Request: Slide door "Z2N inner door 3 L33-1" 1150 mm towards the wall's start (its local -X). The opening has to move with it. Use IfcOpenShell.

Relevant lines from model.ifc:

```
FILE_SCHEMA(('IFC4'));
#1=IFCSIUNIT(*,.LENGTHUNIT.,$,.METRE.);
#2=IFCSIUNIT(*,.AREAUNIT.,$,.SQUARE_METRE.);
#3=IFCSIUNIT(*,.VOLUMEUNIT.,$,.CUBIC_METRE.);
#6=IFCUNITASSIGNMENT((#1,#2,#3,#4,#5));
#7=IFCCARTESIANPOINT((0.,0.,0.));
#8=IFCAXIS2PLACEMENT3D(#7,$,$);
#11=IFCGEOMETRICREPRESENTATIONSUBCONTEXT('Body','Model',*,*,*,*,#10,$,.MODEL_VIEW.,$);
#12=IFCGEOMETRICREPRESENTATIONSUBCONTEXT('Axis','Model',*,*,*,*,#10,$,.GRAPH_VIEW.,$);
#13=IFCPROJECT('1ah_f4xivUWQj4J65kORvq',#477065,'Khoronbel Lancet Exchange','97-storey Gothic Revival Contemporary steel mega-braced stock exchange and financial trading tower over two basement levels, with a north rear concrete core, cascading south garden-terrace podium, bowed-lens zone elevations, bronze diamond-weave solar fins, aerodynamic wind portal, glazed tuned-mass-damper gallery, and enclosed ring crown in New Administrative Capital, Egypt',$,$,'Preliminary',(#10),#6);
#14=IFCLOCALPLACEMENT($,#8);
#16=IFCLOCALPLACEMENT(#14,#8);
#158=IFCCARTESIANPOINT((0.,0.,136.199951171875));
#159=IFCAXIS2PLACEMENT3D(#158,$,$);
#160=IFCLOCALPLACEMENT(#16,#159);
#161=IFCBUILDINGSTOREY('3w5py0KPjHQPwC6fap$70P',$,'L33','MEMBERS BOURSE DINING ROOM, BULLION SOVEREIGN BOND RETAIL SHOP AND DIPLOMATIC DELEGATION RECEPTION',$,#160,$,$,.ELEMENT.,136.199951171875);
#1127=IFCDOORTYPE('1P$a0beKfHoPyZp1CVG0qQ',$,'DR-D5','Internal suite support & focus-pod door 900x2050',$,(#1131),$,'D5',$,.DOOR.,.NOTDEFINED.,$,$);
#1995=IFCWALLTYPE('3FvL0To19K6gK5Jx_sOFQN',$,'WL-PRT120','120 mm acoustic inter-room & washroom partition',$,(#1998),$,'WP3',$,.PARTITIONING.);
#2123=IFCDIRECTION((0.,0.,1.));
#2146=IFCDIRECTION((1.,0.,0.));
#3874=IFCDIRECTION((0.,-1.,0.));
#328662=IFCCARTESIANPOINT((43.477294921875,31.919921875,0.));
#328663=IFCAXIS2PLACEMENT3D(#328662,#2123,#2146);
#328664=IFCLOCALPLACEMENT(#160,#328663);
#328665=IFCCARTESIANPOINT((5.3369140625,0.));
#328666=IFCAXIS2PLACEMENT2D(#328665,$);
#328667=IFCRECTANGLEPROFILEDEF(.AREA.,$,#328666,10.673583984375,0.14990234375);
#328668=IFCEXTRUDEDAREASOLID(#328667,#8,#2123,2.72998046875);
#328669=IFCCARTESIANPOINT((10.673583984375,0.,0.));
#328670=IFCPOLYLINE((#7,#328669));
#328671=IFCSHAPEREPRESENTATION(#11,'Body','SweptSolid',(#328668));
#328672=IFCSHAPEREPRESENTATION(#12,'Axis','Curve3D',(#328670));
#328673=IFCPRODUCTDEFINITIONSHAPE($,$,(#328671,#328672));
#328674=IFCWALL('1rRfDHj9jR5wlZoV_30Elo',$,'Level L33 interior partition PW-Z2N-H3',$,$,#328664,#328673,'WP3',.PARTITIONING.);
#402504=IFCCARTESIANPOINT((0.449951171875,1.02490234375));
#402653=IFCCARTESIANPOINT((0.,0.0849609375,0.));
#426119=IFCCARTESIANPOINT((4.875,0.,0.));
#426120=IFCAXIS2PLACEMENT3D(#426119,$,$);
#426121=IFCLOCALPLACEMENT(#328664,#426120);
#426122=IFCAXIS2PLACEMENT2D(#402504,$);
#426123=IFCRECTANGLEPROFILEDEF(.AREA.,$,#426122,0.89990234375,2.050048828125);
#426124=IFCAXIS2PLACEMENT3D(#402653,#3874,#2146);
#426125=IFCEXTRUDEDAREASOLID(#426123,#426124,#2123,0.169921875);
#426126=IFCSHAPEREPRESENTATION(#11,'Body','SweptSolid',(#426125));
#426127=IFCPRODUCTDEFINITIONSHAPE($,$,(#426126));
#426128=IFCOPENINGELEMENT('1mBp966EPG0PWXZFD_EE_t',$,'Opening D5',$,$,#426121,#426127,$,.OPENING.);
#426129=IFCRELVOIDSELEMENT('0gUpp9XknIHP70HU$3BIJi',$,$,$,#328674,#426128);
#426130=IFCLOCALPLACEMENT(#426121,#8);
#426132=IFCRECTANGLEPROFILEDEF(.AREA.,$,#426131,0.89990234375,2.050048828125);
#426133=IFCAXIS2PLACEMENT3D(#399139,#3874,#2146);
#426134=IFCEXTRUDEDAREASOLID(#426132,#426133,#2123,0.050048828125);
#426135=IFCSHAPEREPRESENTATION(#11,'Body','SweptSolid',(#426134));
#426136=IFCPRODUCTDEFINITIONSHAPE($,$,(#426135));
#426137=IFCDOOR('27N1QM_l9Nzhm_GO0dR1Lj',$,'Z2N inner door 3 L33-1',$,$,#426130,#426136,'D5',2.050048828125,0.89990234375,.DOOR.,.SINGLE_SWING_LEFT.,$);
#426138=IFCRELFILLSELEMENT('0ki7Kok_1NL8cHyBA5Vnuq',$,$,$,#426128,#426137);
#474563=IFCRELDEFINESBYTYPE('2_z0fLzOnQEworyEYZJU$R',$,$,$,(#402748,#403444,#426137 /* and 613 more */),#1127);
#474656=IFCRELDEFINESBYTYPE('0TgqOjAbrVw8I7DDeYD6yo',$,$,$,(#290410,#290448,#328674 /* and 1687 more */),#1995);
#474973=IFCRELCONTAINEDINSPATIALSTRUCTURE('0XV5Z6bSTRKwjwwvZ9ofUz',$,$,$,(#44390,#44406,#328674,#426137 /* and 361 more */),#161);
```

```python
import ifcopenshell
import ifcopenshell.api.geometry
import ifcopenshell.util.placement
import ifcopenshell.util.unit

model = ifcopenshell.open("model.ifc")
unit_scale = ifcopenshell.util.unit.calculate_unit_scale(model)

door = model.by_id(426137)
opening = door.FillsVoids[0].RelatingOpeningElement
wall = opening.VoidsElements[0].RelatingBuildingElement

wall_matrix = ifcopenshell.util.placement.get_local_placement(wall.ObjectPlacement)
shift = wall_matrix[:3, 0] * -1.15 / unit_scale
before = ifcopenshell.util.placement.get_local_placement(door.ObjectPlacement)[:3, 3].copy()

# The door is placed relative to its opening, so it follows when the opening moves.
matrix = ifcopenshell.util.placement.get_local_placement(opening.ObjectPlacement)
matrix[:3, 3] += shift
ifcopenshell.api.geometry.edit_object_placement(
    model, product=opening, matrix=matrix, is_si=False, should_transform_children=True
)

after = ifcopenshell.util.placement.get_local_placement(door.ObjectPlacement)[:3, 3]
print("door moved by", (after - before).round(3) + 0.0)

model.write("model_rev.ifc")
```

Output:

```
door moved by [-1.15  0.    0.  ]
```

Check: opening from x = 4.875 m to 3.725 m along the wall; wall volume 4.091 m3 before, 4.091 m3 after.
